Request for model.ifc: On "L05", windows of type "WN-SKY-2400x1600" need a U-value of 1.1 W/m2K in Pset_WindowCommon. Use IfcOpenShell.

First a look at what the model holds.

```python
import ifcopenshell
import ifcopenshell.util.element

model = ifcopenshell.open("model.ifc")
print(model.schema)
storey = next(s for s in model.by_type("IfcBuildingStorey") if s.Name == "L05")
windows = [e for e in ifcopenshell.util.element.get_decomposition(storey) if e.is_a("IfcWindow")]
seen = {}
for e in windows:
    element_type = ifcopenshell.util.element.get_type(e)
    key = (element_type.Name if element_type != e and element_type else None, ifcopenshell.util.element.get_pset(e, "Pset_WindowCommon", "ThermalTransmittance"))
    seen[key] = seen.get(key, 0) + 1
for (name, value), count in sorted(seen.items(), key=str):
    print(count, "x", name, "|", value)
```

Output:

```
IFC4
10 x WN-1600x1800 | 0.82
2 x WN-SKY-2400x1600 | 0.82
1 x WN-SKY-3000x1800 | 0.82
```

```python
import ifcopenshell
import ifcopenshell.api.pset
import ifcopenshell.util.element

model = ifcopenshell.open("model.ifc")

storey = next(s for s in model.by_type("IfcBuildingStorey") if s.Name == "L05")
windows = [e for e in ifcopenshell.util.element.get_decomposition(storey) if e.is_a("IfcWindow")]

count = 0
for e in windows:
    element_type = ifcopenshell.util.element.get_type(e)
    if element_type in (None, e) or element_type.Name != "WN-SKY-2400x1600":
        continue
    # add_pset returns the element's existing set when there is one.
    pset = ifcopenshell.api.pset.add_pset(model, product=e, name="Pset_WindowCommon")
    ifcopenshell.api.pset.edit_pset(model, pset=pset, properties={"ThermalTransmittance": 1.1})
    count += 1

print(count, "windows updated")

model.write("model-out.ifc")
```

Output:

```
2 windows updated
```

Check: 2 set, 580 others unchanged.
